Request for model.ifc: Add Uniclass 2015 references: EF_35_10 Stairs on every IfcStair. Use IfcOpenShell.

First a look at what the model holds.

```python
import ifcopenshell

model = ifcopenshell.open("model.ifc")
print(model.schema)
print("classifications:", [c.Name for c in model.by_type("IfcClassification")])
for ifc_class in ("IfcDoor", "IfcRoof", "IfcStair", "IfcWall", "IfcWindow"):
    print(ifc_class, len(model.by_type(ifc_class)))
```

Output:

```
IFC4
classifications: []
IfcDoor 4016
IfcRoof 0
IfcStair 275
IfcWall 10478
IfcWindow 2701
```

```python
import ifcopenshell
import ifcopenshell.api.classification

model = ifcopenshell.open("model.ifc")

system = ifcopenshell.api.classification.add_classification(model, classification="Uniclass 2015")

codes = {
    "IfcStair": ("EF_35_10", "Stairs"),
}
for ifc_class, (code, name) in codes.items():
    products = model.by_type(ifc_class)
    ifcopenshell.api.classification.add_reference(
        model, products=products, classification=system, identification=code, name=name
    )
    print(code, len(products))

model.write("model_updated.ifc")
```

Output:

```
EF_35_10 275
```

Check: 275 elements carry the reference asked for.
